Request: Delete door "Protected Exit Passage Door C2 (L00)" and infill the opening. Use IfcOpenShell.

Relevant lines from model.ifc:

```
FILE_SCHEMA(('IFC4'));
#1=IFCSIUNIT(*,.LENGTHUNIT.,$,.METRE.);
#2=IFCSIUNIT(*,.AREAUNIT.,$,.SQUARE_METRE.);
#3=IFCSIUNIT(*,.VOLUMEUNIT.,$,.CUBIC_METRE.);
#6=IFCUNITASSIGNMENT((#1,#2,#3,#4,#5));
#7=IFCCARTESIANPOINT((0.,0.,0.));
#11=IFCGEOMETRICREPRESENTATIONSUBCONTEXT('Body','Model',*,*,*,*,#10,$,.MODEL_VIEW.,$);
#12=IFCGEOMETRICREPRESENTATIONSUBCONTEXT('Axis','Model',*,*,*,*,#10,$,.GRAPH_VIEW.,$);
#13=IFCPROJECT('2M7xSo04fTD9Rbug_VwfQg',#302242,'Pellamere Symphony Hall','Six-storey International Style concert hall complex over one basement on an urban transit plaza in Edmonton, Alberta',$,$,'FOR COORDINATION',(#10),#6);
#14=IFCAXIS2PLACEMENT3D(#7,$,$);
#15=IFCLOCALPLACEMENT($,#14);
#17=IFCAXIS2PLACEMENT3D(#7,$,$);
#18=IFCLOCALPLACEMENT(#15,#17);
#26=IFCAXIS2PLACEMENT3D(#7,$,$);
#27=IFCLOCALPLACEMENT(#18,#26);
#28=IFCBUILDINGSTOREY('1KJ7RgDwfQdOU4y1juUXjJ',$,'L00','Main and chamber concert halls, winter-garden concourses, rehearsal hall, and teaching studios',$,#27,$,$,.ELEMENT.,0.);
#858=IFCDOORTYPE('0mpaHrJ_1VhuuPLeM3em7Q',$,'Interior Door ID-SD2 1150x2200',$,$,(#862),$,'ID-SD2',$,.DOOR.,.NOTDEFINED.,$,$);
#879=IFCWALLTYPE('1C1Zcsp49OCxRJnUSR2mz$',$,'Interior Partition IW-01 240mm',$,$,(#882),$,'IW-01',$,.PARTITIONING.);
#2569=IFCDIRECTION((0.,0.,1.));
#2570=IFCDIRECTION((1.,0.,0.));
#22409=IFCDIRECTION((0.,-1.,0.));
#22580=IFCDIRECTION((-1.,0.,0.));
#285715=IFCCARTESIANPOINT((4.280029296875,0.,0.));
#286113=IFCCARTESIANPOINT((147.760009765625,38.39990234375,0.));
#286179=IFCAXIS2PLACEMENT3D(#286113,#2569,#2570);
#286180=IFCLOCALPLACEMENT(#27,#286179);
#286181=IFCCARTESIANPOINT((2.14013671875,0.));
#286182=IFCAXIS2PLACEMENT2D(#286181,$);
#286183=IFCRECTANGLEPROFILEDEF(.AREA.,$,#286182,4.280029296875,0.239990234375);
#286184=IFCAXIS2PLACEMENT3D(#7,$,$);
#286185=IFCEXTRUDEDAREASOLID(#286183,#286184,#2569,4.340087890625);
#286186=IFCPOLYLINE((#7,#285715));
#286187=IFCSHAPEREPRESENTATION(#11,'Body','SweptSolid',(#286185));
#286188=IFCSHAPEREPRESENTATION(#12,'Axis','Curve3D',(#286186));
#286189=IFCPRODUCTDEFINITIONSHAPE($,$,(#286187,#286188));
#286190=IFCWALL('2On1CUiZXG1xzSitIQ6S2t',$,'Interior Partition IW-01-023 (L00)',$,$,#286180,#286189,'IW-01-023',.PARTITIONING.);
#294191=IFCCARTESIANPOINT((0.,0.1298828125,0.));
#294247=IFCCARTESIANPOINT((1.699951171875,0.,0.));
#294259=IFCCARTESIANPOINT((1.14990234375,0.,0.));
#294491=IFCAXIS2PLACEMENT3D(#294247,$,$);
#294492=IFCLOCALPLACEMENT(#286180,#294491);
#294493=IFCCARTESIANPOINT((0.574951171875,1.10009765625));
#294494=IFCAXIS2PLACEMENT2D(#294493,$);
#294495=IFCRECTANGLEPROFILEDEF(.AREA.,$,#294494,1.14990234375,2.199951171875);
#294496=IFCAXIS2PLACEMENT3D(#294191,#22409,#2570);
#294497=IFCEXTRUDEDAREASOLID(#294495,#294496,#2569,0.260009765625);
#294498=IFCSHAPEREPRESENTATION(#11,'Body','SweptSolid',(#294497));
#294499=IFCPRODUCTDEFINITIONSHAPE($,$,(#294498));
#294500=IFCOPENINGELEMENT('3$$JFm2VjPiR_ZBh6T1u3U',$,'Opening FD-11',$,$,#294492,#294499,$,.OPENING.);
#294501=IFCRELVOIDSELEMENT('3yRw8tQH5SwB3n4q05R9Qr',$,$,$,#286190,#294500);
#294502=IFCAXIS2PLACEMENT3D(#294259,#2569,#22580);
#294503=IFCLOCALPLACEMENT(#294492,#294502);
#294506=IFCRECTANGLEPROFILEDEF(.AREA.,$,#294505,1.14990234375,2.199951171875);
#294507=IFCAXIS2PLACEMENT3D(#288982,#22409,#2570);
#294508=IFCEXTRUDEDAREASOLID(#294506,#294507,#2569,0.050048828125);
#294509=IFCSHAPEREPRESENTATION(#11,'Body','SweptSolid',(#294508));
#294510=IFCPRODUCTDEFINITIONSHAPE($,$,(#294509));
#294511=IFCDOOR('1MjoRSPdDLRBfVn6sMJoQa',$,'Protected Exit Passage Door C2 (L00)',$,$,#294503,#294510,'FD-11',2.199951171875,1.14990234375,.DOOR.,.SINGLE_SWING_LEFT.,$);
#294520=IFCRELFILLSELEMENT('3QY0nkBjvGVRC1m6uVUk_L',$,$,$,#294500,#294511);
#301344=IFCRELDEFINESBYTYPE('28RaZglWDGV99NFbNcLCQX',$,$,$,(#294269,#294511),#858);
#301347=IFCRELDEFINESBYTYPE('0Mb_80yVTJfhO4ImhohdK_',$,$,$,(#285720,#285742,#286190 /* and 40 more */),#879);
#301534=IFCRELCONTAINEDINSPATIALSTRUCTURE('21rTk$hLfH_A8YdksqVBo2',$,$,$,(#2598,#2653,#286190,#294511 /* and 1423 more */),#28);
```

```python
import ifcopenshell
import ifcopenshell.api.feature
import ifcopenshell.api.root
import ifcopenshell.geom
import ifcopenshell.util.shape

model = ifcopenshell.open("model.ifc")
settings = ifcopenshell.geom.settings()


def volume(element):
    """Net volume in cubic metres, openings subtracted."""
    shape = ifcopenshell.geom.create_shape(settings, element)
    return ifcopenshell.util.shape.get_volume(shape.geometry)


door = model.by_guid("1MjoRSPdDLRBfVn6sMJoQa")
opening = door.FillsVoids[0].RelatingOpeningElement
wall = opening.VoidsElements[0].RelatingBuildingElement
before = volume(wall)

ifcopenshell.api.root.remove_product(model, product=door)
ifcopenshell.api.feature.remove_feature(model, feature=opening)

after = volume(wall)

print(f"wall volume {before:.3f} -> {after:.3f} m3")

model.write("model-out.ifc")
```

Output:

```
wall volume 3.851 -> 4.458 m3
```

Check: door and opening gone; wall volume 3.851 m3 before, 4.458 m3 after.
